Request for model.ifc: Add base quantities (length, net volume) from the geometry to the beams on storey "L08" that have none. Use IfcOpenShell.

First a look at what the model holds.

```python
import ifcopenshell
import ifcopenshell.util.element
import ifcopenshell.util.unit

model = ifcopenshell.open("model.ifc")
print(model.schema)
for unit_type in ("LENGTHUNIT", "AREAUNIT", "VOLUMEUNIT"):
    print(unit_type, ifcopenshell.util.unit.calculate_unit_scale(model, unit_type))
storey = next(s for s in model.by_type("IfcBuildingStorey") if s.Name == "L08")
beams = [e for e in ifcopenshell.util.element.get_decomposition(storey) if e.is_a("IfcBeam")]
for e in sorted(beams, key=lambda e: e.id()):
    print(e.id(), e.is_a(), e.Name, list(ifcopenshell.util.element.get_psets(e, qtos_only=True)), sep=" | ")
```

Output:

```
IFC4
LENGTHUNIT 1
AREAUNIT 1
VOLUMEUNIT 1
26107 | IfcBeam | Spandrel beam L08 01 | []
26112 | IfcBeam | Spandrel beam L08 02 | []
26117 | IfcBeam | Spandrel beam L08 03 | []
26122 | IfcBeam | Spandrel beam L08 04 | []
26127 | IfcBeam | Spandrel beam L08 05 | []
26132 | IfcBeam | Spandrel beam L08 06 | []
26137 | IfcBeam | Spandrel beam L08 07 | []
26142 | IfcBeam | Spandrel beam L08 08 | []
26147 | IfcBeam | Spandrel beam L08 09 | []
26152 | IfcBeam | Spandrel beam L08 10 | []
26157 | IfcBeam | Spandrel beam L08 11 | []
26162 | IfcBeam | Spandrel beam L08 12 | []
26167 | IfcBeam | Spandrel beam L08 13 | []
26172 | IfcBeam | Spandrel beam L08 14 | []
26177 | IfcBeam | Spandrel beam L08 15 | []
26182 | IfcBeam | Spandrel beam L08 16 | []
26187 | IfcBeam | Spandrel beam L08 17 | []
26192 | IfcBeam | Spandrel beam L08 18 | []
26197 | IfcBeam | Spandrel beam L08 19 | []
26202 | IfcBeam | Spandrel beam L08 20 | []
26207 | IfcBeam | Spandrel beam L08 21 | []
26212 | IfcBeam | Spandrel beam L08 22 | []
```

```python
import ifcopenshell
import ifcopenshell.api.pset
import ifcopenshell.geom
import ifcopenshell.util.element
import ifcopenshell.util.shape
import ifcopenshell.util.unit

model = ifcopenshell.open("model.ifc")
unit_scale = ifcopenshell.util.unit.calculate_unit_scale(model)
volume_scale = ifcopenshell.util.unit.calculate_unit_scale(model, "VOLUMEUNIT")
settings = ifcopenshell.geom.settings()

storey = next(s for s in model.by_type("IfcBuildingStorey") if s.Name == "L08")
beams = [e for e in ifcopenshell.util.element.get_decomposition(storey) if e.is_a("IfcBeam")]

for e in sorted(beams, key=lambda e: e.id()):
    if ifcopenshell.util.element.get_psets(e, qtos_only=True, should_inherit=False):
        continue
    # Geometry comes back in metres, in the element's own axes.
    shape = ifcopenshell.geom.create_shape(settings, e)
    values = {
        "Length": ifcopenshell.util.shape.get_max_xyz(shape.geometry) / unit_scale,
        "NetVolume": ifcopenshell.util.shape.get_volume(shape.geometry) / volume_scale,
    }
    qto = ifcopenshell.api.pset.add_qto(model, product=e, name="Qto_BeamBaseQuantities")
    ifcopenshell.api.pset.edit_qto(model, qto=qto, properties=values)
    print(e.id(), {k: round(v, 3) for k, v in values.items()})

model.write("model_updated.ifc")
```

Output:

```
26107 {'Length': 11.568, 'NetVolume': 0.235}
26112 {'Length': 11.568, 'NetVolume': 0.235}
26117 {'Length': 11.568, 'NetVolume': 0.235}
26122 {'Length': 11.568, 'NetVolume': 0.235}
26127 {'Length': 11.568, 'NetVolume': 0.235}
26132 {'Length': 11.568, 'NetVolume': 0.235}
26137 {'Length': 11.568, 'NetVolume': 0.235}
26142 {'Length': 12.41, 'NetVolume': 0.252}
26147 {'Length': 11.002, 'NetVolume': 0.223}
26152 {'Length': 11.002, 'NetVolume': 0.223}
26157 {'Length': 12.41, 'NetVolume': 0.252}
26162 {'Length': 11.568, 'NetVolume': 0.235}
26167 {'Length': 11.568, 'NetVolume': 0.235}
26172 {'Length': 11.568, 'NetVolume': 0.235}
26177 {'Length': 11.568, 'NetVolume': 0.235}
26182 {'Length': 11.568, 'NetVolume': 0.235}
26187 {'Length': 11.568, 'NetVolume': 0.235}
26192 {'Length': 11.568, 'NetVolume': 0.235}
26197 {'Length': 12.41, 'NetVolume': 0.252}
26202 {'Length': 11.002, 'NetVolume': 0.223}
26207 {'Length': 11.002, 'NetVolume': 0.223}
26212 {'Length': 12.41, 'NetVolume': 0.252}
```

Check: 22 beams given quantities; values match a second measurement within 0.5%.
